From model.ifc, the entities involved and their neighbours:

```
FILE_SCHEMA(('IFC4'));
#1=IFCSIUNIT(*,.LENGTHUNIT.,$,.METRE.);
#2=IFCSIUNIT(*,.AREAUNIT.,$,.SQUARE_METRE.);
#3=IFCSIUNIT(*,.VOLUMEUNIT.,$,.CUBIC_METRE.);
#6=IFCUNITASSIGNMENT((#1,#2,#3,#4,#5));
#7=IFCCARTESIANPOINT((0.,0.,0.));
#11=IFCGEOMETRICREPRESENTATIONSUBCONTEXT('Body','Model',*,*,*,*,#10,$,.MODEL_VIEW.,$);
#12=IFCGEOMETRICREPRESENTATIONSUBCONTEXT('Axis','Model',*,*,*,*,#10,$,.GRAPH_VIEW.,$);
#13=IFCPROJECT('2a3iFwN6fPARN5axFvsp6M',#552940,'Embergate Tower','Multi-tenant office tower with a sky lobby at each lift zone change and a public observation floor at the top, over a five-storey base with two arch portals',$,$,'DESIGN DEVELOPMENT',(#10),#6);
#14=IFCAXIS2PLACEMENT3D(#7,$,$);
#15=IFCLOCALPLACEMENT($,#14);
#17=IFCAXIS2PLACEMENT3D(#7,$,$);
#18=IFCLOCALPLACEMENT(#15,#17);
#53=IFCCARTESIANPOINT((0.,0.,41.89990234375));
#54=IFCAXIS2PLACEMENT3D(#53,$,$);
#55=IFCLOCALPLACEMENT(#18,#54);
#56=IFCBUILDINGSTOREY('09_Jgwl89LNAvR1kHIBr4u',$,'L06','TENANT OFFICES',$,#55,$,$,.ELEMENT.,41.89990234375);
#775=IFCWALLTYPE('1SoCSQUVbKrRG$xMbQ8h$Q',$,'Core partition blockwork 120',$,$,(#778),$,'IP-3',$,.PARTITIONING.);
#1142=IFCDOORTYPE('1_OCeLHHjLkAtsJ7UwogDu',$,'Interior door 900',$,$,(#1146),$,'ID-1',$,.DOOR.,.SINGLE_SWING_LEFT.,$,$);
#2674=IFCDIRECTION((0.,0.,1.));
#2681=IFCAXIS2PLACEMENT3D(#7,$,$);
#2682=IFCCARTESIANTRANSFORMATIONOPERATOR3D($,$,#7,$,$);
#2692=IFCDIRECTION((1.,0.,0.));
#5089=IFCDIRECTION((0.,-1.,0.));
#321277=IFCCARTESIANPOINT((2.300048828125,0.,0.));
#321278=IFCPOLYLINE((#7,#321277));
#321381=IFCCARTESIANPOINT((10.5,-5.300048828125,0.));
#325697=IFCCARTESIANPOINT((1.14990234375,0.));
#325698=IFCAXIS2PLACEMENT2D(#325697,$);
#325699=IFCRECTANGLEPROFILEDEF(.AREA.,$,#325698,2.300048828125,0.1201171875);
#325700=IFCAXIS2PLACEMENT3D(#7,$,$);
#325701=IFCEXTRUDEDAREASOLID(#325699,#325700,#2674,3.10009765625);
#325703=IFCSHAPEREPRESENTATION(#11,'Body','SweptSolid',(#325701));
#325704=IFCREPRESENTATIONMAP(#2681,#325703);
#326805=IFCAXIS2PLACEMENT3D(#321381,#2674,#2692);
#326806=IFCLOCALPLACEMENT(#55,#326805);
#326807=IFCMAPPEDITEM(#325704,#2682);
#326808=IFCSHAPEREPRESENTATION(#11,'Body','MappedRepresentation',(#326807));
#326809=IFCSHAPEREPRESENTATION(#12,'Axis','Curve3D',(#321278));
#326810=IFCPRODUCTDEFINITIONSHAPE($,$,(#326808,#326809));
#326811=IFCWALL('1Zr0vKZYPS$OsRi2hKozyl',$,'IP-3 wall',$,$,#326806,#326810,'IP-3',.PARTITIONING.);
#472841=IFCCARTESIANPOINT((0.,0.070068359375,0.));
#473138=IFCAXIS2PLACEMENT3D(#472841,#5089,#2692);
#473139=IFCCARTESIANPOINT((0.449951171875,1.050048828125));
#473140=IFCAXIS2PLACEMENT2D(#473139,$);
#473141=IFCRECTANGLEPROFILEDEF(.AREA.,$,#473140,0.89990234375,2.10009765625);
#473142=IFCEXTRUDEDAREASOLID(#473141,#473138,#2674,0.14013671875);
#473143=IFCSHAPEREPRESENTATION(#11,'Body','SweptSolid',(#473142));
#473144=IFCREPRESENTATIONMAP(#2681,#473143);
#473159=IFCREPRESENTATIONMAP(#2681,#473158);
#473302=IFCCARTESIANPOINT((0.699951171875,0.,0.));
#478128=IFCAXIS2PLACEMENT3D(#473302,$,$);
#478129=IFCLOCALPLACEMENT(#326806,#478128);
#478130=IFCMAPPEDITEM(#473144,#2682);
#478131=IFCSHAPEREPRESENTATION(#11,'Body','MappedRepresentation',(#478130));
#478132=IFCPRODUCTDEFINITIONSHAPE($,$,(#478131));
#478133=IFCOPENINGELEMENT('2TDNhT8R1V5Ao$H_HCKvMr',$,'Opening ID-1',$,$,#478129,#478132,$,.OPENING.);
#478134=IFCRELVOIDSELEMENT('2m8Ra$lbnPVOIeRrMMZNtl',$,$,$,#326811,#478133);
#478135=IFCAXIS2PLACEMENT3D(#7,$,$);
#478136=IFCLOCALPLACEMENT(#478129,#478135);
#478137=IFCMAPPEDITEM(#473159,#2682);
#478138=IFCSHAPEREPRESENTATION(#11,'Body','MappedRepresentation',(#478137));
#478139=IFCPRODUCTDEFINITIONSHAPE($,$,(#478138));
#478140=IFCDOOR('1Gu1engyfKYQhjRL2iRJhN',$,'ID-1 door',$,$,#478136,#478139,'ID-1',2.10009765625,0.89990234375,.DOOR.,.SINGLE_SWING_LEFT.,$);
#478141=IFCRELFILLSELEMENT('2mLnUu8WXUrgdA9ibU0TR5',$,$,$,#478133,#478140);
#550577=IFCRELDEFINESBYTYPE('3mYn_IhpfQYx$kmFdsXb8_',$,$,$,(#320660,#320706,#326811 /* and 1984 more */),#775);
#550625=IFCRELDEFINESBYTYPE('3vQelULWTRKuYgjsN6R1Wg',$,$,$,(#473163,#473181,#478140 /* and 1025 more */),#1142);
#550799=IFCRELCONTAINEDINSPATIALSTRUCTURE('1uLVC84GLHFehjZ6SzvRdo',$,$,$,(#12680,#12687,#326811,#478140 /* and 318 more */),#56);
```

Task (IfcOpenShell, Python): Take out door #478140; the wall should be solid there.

```python
import ifcopenshell
import ifcopenshell.api.feature
import ifcopenshell.api.root
import ifcopenshell.geom
import ifcopenshell.util.shape

model = ifcopenshell.open("model.ifc")
settings = ifcopenshell.geom.settings()


def volume(element):
    """Net volume in cubic metres, openings subtracted."""
    shape = ifcopenshell.geom.create_shape(settings, element)
    return ifcopenshell.util.shape.get_volume(shape.geometry)


door = model.by_guid("1Gu1engyfKYQhjRL2iRJhN")
opening = door.FillsVoids[0].RelatingOpeningElement
wall = opening.VoidsElements[0].RelatingBuildingElement
before = volume(wall)

ifcopenshell.api.root.remove_product(model, product=door)
ifcopenshell.api.feature.remove_feature(model, feature=opening)

after = volume(wall)

print(f"wall volume {before:.3f} -> {after:.3f} m3")

model.write("model-out.ifc")
```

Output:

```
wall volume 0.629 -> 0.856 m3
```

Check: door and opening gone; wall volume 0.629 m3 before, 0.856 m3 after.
